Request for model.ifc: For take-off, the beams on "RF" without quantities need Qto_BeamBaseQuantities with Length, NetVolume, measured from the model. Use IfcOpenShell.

First a look at what the model holds.

```python
import ifcopenshell
import ifcopenshell.util.element
import ifcopenshell.util.unit

model = ifcopenshell.open("model.ifc")
print(model.schema)
for unit_type in ("LENGTHUNIT", "AREAUNIT", "VOLUMEUNIT"):
    print(unit_type, ifcopenshell.util.unit.calculate_unit_scale(model, unit_type))
storey = next(s for s in model.by_type("IfcBuildingStorey") if s.Name == "RF")
beams = [e for e in ifcopenshell.util.element.get_decomposition(storey) if e.is_a("IfcBeam")]
for e in sorted(beams, key=lambda e: e.id()):
    print(e.id(), e.is_a(), e.Name, list(ifcopenshell.util.element.get_psets(e, qtos_only=True)), sep=" | ")
```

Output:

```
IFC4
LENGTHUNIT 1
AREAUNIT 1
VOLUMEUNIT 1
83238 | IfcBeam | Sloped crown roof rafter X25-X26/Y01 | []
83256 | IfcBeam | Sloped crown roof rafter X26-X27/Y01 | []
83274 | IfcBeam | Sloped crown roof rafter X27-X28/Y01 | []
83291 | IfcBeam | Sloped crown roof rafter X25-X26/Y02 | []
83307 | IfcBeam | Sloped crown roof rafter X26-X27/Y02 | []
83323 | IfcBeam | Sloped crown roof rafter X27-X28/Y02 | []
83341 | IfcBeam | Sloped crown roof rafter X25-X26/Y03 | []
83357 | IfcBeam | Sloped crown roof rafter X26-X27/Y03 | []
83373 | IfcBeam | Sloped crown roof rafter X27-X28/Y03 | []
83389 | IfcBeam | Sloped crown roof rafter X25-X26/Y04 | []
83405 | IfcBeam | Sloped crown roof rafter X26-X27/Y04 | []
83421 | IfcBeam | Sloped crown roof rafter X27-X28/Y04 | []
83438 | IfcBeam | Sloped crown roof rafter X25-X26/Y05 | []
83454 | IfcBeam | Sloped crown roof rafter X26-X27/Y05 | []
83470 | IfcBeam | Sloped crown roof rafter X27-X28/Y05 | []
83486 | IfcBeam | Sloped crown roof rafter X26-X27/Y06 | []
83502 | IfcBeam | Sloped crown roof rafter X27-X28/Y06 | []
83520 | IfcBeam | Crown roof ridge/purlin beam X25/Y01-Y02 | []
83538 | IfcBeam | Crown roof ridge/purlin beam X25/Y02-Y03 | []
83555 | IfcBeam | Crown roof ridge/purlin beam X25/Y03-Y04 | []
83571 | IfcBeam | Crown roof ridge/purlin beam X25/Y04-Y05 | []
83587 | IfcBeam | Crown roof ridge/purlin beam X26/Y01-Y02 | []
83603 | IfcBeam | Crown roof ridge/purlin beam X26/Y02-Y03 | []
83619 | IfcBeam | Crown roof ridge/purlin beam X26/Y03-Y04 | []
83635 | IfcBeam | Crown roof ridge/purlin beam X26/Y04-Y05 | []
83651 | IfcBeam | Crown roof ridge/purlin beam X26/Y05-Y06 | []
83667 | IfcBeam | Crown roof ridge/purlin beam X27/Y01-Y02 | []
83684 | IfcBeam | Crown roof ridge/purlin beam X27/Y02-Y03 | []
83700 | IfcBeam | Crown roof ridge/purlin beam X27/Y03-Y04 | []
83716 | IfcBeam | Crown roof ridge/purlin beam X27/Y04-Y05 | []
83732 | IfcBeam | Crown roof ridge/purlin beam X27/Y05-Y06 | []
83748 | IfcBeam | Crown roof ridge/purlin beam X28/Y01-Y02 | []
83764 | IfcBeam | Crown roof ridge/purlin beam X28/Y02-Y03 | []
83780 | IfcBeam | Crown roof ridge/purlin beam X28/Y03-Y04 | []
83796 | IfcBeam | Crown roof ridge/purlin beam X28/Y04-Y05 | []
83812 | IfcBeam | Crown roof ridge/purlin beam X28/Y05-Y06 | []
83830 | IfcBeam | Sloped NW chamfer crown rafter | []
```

```python
import ifcopenshell
import ifcopenshell.api.pset
import ifcopenshell.geom
import ifcopenshell.util.element
import ifcopenshell.util.shape
import ifcopenshell.util.unit

model = ifcopenshell.open("model.ifc")
unit_scale = ifcopenshell.util.unit.calculate_unit_scale(model)
volume_scale = ifcopenshell.util.unit.calculate_unit_scale(model, "VOLUMEUNIT")
settings = ifcopenshell.geom.settings()

storey = next(s for s in model.by_type("IfcBuildingStorey") if s.Name == "RF")
beams = [e for e in ifcopenshell.util.element.get_decomposition(storey) if e.is_a("IfcBeam")]

for e in sorted(beams, key=lambda e: e.id()):
    if ifcopenshell.util.element.get_psets(e, qtos_only=True, should_inherit=False):
        continue
    # Geometry comes back in metres, in the element's own axes.
    shape = ifcopenshell.geom.create_shape(settings, e)
    values = {
        "Length": ifcopenshell.util.shape.get_max_xyz(shape.geometry) / unit_scale,
        "NetVolume": ifcopenshell.util.shape.get_volume(shape.geometry) / volume_scale,
    }
    qto = ifcopenshell.api.pset.add_qto(model, product=e, name="Qto_BeamBaseQuantities")
    ifcopenshell.api.pset.edit_qto(model, qto=qto, properties=values)
    print(e.id(), {k: round(v, 3) for k, v in values.items()})

model.write("model_edited.ifc")
```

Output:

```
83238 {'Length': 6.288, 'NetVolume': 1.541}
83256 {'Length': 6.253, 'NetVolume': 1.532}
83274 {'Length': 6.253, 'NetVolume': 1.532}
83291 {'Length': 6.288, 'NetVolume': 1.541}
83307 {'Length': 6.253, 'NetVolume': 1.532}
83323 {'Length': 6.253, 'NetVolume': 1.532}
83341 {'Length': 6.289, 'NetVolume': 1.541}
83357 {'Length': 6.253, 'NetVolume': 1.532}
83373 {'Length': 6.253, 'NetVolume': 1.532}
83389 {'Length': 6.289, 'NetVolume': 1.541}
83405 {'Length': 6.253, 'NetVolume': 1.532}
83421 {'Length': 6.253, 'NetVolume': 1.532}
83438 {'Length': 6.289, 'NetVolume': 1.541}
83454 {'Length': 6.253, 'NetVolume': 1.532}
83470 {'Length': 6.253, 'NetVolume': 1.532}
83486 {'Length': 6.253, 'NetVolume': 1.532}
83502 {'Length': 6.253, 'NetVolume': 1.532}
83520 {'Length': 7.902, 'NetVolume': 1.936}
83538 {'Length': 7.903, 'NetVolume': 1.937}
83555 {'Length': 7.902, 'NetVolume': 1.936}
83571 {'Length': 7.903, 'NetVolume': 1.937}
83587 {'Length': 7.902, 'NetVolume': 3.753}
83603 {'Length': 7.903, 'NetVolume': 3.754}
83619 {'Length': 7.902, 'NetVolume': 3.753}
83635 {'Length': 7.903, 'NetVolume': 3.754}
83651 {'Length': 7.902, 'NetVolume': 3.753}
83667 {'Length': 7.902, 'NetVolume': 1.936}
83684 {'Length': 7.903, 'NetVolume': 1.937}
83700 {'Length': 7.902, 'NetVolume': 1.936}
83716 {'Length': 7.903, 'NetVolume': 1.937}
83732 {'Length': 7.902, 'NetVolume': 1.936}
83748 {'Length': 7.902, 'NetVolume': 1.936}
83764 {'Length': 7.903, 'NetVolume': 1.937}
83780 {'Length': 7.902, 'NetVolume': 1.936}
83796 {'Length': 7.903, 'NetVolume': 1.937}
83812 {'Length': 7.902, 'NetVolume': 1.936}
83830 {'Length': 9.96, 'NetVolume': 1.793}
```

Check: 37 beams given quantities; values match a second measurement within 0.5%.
